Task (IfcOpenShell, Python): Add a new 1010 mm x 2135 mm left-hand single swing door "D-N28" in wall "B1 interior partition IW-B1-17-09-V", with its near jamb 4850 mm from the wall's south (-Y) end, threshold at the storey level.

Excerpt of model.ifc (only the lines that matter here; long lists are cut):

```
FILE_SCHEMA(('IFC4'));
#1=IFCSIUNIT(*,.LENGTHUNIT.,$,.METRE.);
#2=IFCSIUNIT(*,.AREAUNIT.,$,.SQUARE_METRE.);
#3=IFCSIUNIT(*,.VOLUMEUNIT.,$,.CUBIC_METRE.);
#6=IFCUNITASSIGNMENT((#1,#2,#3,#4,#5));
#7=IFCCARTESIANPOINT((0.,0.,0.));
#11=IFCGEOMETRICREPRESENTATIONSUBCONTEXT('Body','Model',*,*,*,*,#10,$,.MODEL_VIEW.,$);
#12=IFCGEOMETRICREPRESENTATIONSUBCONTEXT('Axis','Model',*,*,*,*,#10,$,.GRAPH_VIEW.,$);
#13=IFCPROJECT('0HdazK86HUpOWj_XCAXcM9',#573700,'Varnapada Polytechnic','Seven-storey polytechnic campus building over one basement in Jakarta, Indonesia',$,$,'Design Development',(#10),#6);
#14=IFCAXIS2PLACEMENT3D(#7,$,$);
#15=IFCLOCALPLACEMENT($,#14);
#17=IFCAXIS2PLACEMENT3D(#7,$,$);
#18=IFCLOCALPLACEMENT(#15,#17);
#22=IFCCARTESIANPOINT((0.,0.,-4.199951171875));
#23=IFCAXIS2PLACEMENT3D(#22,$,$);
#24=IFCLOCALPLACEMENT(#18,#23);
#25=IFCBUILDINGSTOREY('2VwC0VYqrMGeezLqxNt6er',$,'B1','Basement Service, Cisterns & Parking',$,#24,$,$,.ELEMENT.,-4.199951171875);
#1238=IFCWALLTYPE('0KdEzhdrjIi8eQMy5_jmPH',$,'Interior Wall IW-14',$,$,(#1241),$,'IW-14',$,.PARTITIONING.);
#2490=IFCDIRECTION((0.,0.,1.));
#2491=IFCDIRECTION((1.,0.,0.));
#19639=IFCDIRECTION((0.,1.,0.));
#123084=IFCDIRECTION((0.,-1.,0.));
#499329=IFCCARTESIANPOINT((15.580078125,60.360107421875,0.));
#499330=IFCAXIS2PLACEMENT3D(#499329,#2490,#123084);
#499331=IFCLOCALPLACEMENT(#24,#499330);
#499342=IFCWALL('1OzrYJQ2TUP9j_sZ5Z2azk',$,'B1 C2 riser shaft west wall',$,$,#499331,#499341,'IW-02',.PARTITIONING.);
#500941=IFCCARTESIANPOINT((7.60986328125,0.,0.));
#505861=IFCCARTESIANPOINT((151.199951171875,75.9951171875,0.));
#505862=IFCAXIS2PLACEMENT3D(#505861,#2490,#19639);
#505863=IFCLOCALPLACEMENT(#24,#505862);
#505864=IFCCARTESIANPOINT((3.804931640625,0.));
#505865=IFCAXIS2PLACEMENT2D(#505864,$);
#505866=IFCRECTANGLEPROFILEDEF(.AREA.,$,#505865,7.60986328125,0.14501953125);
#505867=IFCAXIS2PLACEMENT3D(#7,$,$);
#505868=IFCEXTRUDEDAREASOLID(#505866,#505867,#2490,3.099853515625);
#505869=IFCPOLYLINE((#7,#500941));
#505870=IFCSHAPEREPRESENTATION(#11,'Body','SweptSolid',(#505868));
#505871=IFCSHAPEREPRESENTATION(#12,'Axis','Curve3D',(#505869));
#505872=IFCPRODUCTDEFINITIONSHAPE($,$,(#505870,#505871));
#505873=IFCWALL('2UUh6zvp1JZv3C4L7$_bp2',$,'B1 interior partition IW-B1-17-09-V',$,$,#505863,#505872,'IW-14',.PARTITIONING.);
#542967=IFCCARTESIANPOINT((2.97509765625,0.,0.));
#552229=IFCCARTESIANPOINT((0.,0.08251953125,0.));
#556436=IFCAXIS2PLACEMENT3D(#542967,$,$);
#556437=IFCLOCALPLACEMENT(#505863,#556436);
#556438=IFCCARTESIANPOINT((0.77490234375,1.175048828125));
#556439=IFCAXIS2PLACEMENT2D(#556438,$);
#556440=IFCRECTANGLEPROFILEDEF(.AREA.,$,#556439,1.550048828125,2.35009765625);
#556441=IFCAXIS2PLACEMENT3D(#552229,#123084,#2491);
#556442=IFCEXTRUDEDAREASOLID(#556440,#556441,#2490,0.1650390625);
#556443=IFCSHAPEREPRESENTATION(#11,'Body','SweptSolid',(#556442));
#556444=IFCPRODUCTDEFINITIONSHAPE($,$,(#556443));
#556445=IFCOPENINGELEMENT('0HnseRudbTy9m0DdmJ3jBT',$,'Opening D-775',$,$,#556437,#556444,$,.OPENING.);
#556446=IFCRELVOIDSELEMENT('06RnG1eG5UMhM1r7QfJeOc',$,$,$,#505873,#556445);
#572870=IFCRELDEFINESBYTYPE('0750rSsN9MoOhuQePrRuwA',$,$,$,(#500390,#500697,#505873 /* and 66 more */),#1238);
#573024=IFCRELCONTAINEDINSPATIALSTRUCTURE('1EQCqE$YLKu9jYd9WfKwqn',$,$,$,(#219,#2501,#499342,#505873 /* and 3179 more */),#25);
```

```python
import numpy as np
import ifcopenshell
import ifcopenshell.api.feature
import ifcopenshell.api.geometry
import ifcopenshell.api.root
import ifcopenshell.api.spatial
import ifcopenshell.geom
import ifcopenshell.util.element
import ifcopenshell.util.placement
import ifcopenshell.util.representation
import ifcopenshell.util.shape
import ifcopenshell.util.unit

model = ifcopenshell.open("model.ifc")
unit_scale = ifcopenshell.util.unit.calculate_unit_scale(model)
settings = ifcopenshell.geom.settings()


def volume(element):
    """Net volume in cubic metres, openings subtracted."""
    shape = ifcopenshell.geom.create_shape(settings, element)
    return ifcopenshell.util.shape.get_volume(shape.geometry)


wall = model.by_guid("2UUh6zvp1JZv3C4L7$_bp2")
storey = ifcopenshell.util.element.get_container(wall, ifc_class="IfcBuildingStorey")
context = ifcopenshell.util.representation.get_context(model, "Model", "Body", "MODEL_VIEW")
before = volume(wall)

width, height, from_end, sill = 1.01, 2.135, 4.85, 0.0  # metres

# The wall runs along its own X axis, and the end named is its -X end.
wall_shape = ifcopenshell.geom.create_shape(settings, wall)
x, y, z = ifcopenshell.util.shape.get_vertices(wall_shape.geometry).T
start = x.min() + from_end
face, thickness = float(y.min()), float(y.max() - y.min())
wall_matrix = ifcopenshell.util.placement.get_local_placement(wall.ObjectPlacement)
level = ifcopenshell.util.placement.get_local_placement(storey.ObjectPlacement)[2, 3]


def in_wall(x, y):
    """Placement at x, y metres in the wall's axes, at sill height."""
    matrix = wall_matrix.copy()
    matrix[:, 3] = wall_matrix @ np.array([x / unit_scale, y / unit_scale, 0.0, 1.0])
    matrix[2, 3] = level + sill / unit_scale
    return matrix


# Opening: a box that overshoots both wall faces by 50 mm.
opening = ifcopenshell.api.root.create_entity(model, ifc_class="IfcOpeningElement", predefined_type="OPENING")
box = ifcopenshell.api.geometry.add_wall_representation(
    model, context=context, length=width, height=height, thickness=thickness + 0.1
)
ifcopenshell.api.geometry.assign_representation(model, product=opening, representation=box)
ifcopenshell.api.geometry.edit_object_placement(model, product=opening, matrix=in_wall(start, face - 0.05), is_si=False)
ifcopenshell.api.feature.add_feature(model, feature=opening, element=wall)

door = ifcopenshell.api.root.create_entity(model, ifc_class="IfcDoor", name="D-N28", predefined_type="DOOR")
door.OverallWidth, door.OverallHeight = width / unit_scale, height / unit_scale
door.OperationType = "SINGLE_SWING_LEFT"
body = ifcopenshell.api.geometry.add_door_representation(
    model,
    context=context,
    overall_width=door.OverallWidth,
    overall_height=door.OverallHeight,
    operation_type="SINGLE_SWING_LEFT",
    lining_properties={"LiningDepth": thickness / unit_scale, "ThresholdDepth": thickness / unit_scale},
)
ifcopenshell.api.geometry.assign_representation(model, product=door, representation=body)
ifcopenshell.api.spatial.assign_container(model, products=[door], relating_structure=storey)
ifcopenshell.api.feature.add_filling(model, opening=opening, element=door)

# The lining spans the wall, so the door starts at the wall face.
ifcopenshell.api.geometry.edit_object_placement(model, product=door, matrix=in_wall(start, face), is_si=False)

after = volume(wall)

print(f"wall volume {before:.3f} -> {after:.3f} m3")

model.write("model_rev.ifc")
```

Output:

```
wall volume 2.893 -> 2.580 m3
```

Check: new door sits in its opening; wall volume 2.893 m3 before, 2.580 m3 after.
